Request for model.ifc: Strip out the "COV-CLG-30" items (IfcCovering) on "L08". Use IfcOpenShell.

First a look at what the model holds.

```python
import ifcopenshell
import ifcopenshell.util.element

model = ifcopenshell.open("model.ifc")
print(model.schema)
storey = next(s for s in model.by_type("IfcBuildingStorey") if s.Name == "L08")
coverings = [e for e in ifcopenshell.util.element.get_decomposition(storey) if e.is_a("IfcCovering")]
seen = {}
for e in coverings:
    element_type = ifcopenshell.util.element.get_type(e)
    name = element_type.Name if element_type not in (None, e) else None
    seen[name] = seen.get(name, 0) + 1
for name, count in sorted(seen.items(), key=str):
    print(count, "x", name)
```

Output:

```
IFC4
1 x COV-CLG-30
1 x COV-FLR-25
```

```python
import ifcopenshell
import ifcopenshell.api.root
import ifcopenshell.util.element

model = ifcopenshell.open("model.ifc")

storey = next(s for s in model.by_type("IfcBuildingStorey") if s.Name == "L08")
coverings = [e for e in ifcopenshell.util.element.get_decomposition(storey) if e.is_a("IfcCovering")]
targets = [e for e in coverings if (t := ifcopenshell.util.element.get_type(e)) not in (None, e) and t.Name == "COV-CLG-30"]

for e in targets:
    ifcopenshell.api.root.remove_product(model, product=e)
print(len(targets), "removed")

model.write("model_rev.ifc")
```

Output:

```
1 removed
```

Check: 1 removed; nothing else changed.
